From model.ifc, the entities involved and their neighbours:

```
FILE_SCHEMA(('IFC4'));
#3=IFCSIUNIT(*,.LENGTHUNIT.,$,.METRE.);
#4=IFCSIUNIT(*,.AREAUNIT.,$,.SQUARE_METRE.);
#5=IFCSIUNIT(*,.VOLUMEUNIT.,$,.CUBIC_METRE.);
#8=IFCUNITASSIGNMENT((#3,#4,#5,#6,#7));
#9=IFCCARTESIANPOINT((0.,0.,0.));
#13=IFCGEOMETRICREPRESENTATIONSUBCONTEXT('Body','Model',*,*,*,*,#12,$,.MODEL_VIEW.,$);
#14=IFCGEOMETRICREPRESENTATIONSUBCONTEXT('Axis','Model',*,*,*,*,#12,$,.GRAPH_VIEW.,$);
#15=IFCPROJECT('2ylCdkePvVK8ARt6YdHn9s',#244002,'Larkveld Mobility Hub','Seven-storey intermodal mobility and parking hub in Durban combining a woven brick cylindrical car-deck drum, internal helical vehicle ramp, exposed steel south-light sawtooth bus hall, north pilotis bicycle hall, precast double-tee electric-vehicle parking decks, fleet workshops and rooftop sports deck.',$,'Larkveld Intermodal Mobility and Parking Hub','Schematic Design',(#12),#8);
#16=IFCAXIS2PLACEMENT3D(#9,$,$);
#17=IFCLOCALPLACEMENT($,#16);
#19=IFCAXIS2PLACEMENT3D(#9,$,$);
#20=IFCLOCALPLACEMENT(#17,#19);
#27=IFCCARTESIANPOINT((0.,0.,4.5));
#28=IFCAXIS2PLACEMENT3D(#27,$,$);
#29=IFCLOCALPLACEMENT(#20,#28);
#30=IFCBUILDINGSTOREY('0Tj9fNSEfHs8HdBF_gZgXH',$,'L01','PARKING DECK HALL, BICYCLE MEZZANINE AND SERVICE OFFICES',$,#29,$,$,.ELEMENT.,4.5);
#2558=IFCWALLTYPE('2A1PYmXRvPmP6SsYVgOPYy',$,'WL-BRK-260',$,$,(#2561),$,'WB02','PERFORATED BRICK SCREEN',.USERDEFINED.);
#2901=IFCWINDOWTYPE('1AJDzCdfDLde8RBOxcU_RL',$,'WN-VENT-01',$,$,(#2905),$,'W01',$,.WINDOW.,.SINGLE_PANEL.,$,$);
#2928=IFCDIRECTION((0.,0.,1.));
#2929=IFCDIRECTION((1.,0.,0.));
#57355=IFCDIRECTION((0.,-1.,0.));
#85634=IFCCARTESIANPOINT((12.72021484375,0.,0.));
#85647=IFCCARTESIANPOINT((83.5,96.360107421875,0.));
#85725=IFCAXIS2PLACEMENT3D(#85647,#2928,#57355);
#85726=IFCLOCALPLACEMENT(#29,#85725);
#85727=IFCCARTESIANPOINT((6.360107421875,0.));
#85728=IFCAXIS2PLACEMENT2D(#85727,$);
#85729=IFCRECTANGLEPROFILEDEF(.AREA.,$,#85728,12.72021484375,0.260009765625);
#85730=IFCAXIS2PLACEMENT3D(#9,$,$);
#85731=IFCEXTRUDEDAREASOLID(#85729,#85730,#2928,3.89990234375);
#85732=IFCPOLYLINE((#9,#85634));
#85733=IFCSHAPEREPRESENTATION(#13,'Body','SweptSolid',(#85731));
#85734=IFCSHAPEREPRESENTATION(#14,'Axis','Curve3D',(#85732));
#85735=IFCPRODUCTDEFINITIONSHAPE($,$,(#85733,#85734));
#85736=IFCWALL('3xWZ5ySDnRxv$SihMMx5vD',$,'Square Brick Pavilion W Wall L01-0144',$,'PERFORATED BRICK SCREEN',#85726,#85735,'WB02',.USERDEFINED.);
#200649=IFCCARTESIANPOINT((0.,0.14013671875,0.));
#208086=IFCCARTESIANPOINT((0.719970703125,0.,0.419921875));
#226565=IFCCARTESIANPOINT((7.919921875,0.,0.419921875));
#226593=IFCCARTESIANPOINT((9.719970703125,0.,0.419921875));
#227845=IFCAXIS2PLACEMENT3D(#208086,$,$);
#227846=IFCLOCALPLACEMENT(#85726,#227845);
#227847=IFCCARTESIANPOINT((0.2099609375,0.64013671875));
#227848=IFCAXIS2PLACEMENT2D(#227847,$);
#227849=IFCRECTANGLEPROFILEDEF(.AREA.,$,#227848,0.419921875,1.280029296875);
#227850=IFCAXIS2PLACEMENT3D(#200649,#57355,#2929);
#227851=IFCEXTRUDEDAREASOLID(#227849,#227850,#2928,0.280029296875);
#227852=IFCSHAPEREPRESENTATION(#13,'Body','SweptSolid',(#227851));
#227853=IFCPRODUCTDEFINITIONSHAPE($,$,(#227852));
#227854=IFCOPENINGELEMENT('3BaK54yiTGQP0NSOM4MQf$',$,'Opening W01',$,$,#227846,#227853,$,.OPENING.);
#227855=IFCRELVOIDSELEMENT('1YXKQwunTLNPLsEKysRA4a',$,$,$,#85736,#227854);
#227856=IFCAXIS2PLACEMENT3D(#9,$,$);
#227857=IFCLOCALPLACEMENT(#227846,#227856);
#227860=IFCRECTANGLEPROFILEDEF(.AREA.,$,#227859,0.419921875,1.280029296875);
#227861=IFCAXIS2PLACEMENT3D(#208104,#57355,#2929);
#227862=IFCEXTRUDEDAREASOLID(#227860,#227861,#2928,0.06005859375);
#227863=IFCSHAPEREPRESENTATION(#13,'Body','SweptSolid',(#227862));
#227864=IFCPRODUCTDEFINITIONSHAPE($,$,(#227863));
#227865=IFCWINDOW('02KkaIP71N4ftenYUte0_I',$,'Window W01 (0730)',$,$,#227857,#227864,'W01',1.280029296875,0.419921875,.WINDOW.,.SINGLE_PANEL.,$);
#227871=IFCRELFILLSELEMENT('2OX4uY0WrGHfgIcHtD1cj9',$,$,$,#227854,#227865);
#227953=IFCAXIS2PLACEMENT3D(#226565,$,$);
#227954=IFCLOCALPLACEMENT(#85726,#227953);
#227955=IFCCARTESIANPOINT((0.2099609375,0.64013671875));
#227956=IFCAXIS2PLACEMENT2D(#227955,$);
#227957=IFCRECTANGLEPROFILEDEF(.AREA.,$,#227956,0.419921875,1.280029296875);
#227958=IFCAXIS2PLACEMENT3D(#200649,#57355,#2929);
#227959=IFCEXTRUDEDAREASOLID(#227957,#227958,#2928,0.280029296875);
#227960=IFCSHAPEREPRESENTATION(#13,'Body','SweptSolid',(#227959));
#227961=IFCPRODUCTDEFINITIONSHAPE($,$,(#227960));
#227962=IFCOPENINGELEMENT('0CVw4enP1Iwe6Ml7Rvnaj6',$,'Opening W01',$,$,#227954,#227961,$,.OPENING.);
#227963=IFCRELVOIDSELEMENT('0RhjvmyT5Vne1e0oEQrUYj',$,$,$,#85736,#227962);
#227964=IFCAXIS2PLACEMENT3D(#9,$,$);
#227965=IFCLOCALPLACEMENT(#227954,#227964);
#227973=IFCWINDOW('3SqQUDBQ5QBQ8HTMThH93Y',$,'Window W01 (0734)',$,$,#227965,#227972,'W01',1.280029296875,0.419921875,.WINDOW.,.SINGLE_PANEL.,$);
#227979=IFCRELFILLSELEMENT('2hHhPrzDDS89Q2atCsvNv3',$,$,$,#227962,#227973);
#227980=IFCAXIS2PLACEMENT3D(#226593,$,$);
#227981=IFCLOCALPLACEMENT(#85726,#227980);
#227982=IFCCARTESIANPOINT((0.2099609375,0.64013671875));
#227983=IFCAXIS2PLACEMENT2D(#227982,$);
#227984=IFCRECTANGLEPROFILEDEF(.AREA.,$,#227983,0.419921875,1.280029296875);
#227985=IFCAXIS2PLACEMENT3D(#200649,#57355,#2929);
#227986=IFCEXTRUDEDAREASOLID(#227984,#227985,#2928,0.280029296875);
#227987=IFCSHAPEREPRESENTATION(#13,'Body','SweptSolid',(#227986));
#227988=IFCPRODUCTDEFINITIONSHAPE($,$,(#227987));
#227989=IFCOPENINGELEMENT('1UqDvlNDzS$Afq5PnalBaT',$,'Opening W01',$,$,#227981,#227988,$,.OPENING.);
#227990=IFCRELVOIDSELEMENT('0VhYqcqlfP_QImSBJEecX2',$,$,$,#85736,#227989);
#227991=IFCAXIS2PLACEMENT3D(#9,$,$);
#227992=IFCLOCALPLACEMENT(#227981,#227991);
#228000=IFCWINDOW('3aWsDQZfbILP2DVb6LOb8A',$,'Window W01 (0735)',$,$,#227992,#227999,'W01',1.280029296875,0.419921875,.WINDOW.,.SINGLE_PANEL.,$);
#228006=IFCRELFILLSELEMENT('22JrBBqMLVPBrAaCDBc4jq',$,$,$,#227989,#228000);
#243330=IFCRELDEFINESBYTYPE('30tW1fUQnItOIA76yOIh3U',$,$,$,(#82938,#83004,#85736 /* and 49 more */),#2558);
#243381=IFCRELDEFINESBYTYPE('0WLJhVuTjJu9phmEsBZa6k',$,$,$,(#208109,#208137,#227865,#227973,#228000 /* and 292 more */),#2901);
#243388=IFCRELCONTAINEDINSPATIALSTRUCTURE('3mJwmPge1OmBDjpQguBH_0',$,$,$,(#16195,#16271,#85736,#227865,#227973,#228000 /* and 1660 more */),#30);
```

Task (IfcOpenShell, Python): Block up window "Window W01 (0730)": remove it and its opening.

```python
import ifcopenshell
import ifcopenshell.api.feature
import ifcopenshell.api.root
import ifcopenshell.geom
import ifcopenshell.util.shape

model = ifcopenshell.open("model.ifc")
settings = ifcopenshell.geom.settings()


def volume(element):
    """Net volume in cubic metres, openings subtracted."""
    shape = ifcopenshell.geom.create_shape(settings, element)
    return ifcopenshell.util.shape.get_volume(shape.geometry)


window = model.by_guid("02KkaIP71N4ftenYUte0_I")
opening = window.FillsVoids[0].RelatingOpeningElement
wall = opening.VoidsElements[0].RelatingBuildingElement
before = volume(wall)

ifcopenshell.api.root.remove_product(model, product=window)
ifcopenshell.api.feature.remove_feature(model, feature=opening)

after = volume(wall)

print(f"wall volume {before:.3f} -> {after:.3f} m3")

model.write("model_edited.ifc")
```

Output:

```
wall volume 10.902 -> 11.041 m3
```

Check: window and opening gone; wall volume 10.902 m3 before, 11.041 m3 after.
